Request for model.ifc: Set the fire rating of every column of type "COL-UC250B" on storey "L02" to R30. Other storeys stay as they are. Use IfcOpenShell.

First a look at what the model holds.

```python
import ifcopenshell
import ifcopenshell.util.element

model = ifcopenshell.open("model.ifc")
print(model.schema)
storey = next(s for s in model.by_type("IfcBuildingStorey") if s.Name == "L02")
columns = [e for e in ifcopenshell.util.element.get_decomposition(storey) if e.is_a("IfcColumn")]
seen = {}
for e in columns:
    element_type = ifcopenshell.util.element.get_type(e)
    key = (element_type.Name if element_type != e and element_type else None, ifcopenshell.util.element.get_pset(e, "Pset_ColumnCommon", "FireRating"))
    seen[key] = seen.get(key, 0) + 1
for (name, value), count in sorted(seen.items(), key=str):
    print(count, "x", name, "|", value)
```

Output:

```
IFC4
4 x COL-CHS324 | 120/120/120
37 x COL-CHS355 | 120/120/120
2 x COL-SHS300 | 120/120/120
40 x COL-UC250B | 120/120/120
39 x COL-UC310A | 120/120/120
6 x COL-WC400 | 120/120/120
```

```python
import ifcopenshell
import ifcopenshell.api.pset
import ifcopenshell.util.element

model = ifcopenshell.open("model.ifc")

storey = next(s for s in model.by_type("IfcBuildingStorey") if s.Name == "L02")
columns = [e for e in ifcopenshell.util.element.get_decomposition(storey) if e.is_a("IfcColumn")]

count = 0
for e in columns:
    element_type = ifcopenshell.util.element.get_type(e)
    if element_type in (None, e) or element_type.Name != "COL-UC250B":
        continue
    # add_pset returns the element's existing set when there is one.
    pset = ifcopenshell.api.pset.add_pset(model, product=e, name="Pset_ColumnCommon")
    ifcopenshell.api.pset.edit_pset(model, pset=pset, properties={"FireRating": "R30"})
    count += 1

print(count, "columns updated")

model.write("model_v2.ifc")
```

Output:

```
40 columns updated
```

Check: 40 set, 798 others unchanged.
